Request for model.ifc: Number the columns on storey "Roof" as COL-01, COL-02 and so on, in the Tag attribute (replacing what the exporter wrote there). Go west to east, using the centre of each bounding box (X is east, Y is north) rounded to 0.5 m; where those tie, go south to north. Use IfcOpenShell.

First a look at what the model holds.

```python
import ifcopenshell
import ifcopenshell.util.element
import ifcopenshell.util.placement

model = ifcopenshell.open("model.ifc")
print(model.schema)
storey = next(s for s in model.by_type("IfcBuildingStorey") if s.Name == "Roof")
columns = [e for e in ifcopenshell.util.element.get_decomposition(storey) if e.is_a("IfcColumn")]
for e in sorted(columns, key=lambda e: e.id()):
    origin = ifcopenshell.util.placement.get_local_placement(e.ObjectPlacement)[:3, 3]
    print(e.id(), e.Tag, e.Name, origin.round(2) + 0.0, sep=" | ")
```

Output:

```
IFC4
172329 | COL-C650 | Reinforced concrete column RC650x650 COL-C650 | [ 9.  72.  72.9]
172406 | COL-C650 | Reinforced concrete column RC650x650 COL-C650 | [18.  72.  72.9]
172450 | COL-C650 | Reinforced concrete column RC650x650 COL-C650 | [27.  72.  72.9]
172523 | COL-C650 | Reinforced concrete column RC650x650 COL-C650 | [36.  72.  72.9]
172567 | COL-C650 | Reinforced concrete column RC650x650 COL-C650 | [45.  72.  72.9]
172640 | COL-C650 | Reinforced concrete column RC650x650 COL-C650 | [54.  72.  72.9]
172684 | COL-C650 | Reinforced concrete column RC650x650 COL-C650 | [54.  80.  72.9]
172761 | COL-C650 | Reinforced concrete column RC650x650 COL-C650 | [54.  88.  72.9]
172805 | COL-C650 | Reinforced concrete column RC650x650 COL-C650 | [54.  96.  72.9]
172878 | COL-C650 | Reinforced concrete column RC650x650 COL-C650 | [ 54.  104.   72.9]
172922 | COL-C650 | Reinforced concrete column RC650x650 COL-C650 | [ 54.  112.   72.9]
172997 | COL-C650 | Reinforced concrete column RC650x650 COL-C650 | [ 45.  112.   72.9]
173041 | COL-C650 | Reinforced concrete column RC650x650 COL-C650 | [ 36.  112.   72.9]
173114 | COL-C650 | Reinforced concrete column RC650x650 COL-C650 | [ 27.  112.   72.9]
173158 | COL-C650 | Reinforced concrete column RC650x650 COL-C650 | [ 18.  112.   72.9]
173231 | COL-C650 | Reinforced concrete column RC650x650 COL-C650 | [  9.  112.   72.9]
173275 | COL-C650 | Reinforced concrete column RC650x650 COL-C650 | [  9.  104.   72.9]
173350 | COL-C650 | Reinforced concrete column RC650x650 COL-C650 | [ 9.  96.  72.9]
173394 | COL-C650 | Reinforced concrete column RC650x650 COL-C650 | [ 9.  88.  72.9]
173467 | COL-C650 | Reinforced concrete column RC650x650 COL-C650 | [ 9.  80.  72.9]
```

```python
import ifcopenshell
import ifcopenshell.geom
import ifcopenshell.util.element
import ifcopenshell.util.shape

model = ifcopenshell.open("model.ifc")
settings = ifcopenshell.geom.settings()
settings.set("use-world-coords", True)


def centre(element):
    shape = ifcopenshell.geom.create_shape(settings, element)
    return ifcopenshell.util.shape.get_bbox_centroid(shape.geometry)


storey = next(s for s in model.by_type("IfcBuildingStorey") if s.Name == "Roof")
columns = [e for e in ifcopenshell.util.element.get_decomposition(storey) if e.is_a("IfcColumn")]

# Insertion points can sit at a corner or the storey origin, so sort by the geometry (in metres).
centres = {e: centre(e) for e in columns}
columns.sort(key=lambda e: (round(centres[e][0] / 0.5), centres[e][1]))

for i, e in enumerate(columns, start=1):
    number = f"COL-{i:02d}"
    e.Tag = number
    print(e.id(), number)

model.write("model_rev.ifc")
```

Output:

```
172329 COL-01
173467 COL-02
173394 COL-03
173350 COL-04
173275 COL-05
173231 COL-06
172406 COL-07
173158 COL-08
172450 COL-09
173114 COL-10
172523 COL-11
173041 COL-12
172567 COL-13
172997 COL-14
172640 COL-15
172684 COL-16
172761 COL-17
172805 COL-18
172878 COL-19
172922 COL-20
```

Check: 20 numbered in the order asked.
